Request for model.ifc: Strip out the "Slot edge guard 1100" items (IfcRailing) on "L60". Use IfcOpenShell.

First a look at what the model holds.

```python
import ifcopenshell
import ifcopenshell.util.element

model = ifcopenshell.open("model.ifc")
print(model.schema)
storey = next(s for s in model.by_type("IfcBuildingStorey") if s.Name == "L60")
railings = [e for e in ifcopenshell.util.element.get_decomposition(storey) if e.is_a("IfcRailing")]
seen = {}
for e in railings:
    element_type = ifcopenshell.util.element.get_type(e)
    name = element_type.Name if element_type not in (None, e) else None
    seen[name] = seen.get(name, 0) + 1
for name, count in sorted(seen.items(), key=str):
    print(count, "x", name)
```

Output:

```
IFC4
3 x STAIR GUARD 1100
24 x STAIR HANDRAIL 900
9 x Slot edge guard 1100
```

```python
import ifcopenshell
import ifcopenshell.api.root
import ifcopenshell.util.element

model = ifcopenshell.open("model.ifc")

storey = next(s for s in model.by_type("IfcBuildingStorey") if s.Name == "L60")
railings = [e for e in ifcopenshell.util.element.get_decomposition(storey) if e.is_a("IfcRailing")]
targets = [e for e in railings if (t := ifcopenshell.util.element.get_type(e)) not in (None, e) and t.Name == "Slot edge guard 1100"]

for e in targets:
    ifcopenshell.api.root.remove_product(model, product=e)
print(len(targets), "removed")

model.write("model_edited.ifc")
```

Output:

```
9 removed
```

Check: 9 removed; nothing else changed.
